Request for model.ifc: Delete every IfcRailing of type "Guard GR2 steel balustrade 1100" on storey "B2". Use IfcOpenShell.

First a look at what the model holds.

```python
import ifcopenshell
import ifcopenshell.util.element

model = ifcopenshell.open("model.ifc")
print(model.schema)
storey = next(s for s in model.by_type("IfcBuildingStorey") if s.Name == "B2")
railings = [e for e in ifcopenshell.util.element.get_decomposition(storey) if e.is_a("IfcRailing")]
seen = {}
for e in railings:
    element_type = ifcopenshell.util.element.get_type(e)
    name = element_type.Name if element_type not in (None, e) else None
    seen[name] = seen.get(name, 0) + 1
for name, count in sorted(seen.items(), key=str):
    print(count, "x", name)
```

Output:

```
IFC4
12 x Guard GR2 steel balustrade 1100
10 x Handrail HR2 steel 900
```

```python
import ifcopenshell
import ifcopenshell.api.root
import ifcopenshell.util.element

model = ifcopenshell.open("model.ifc")

storey = next(s for s in model.by_type("IfcBuildingStorey") if s.Name == "B2")
railings = [e for e in ifcopenshell.util.element.get_decomposition(storey) if e.is_a("IfcRailing")]
targets = [e for e in railings if (t := ifcopenshell.util.element.get_type(e)) not in (None, e) and t.Name == "Guard GR2 steel balustrade 1100"]

for e in targets:
    ifcopenshell.api.root.remove_product(model, product=e)
print(len(targets), "removed")

model.write("model_updated.ifc")
```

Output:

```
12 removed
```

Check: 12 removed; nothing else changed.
